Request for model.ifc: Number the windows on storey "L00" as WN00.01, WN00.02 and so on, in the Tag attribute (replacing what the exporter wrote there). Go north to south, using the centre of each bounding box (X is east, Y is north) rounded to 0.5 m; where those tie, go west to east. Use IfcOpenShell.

First a look at what the model holds.

```python
import ifcopenshell
import ifcopenshell.util.element
import ifcopenshell.util.placement

model = ifcopenshell.open("model.ifc")
print(model.schema)
storey = next(s for s in model.by_type("IfcBuildingStorey") if s.Name == "L00")
windows = [e for e in ifcopenshell.util.element.get_decomposition(storey) if e.is_a("IfcWindow")]
for e in sorted(windows, key=lambda e: e.id()):
    origin = ifcopenshell.util.placement.get_local_placement(e.ObjectPlacement)[:3, 3]
    print(e.id(), e.Tag, e.Name, origin.round(2) + 0.0, sep=" | ")
```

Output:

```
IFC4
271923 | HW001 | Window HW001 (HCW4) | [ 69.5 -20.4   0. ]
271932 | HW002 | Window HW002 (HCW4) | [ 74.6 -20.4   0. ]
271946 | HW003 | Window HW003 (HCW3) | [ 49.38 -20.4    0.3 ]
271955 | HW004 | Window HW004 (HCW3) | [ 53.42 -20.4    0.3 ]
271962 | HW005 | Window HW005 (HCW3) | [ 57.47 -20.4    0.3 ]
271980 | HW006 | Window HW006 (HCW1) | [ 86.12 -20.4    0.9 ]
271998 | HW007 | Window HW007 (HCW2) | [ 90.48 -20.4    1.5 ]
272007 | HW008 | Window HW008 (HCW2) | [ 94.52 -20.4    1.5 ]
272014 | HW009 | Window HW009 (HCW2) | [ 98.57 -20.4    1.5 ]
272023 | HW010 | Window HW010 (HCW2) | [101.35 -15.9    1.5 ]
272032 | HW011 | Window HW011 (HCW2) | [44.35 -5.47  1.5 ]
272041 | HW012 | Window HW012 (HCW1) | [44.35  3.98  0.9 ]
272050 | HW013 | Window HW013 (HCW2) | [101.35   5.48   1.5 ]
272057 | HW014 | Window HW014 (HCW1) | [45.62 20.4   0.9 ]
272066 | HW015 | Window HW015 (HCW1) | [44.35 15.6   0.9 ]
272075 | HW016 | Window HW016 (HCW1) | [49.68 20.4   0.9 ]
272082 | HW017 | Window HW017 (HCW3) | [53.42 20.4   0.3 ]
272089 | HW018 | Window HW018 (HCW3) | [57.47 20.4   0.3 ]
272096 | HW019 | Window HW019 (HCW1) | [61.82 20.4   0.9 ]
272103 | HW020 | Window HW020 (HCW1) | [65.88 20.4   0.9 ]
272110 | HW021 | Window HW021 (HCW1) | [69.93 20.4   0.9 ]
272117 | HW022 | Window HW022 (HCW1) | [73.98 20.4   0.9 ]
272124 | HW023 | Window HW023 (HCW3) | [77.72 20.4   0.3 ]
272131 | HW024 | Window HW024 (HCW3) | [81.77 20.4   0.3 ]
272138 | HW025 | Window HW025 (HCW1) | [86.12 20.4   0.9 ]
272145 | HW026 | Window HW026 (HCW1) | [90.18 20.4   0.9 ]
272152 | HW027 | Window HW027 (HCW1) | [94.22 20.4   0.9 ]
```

```python
import ifcopenshell
import ifcopenshell.geom
import ifcopenshell.util.element
import ifcopenshell.util.shape

model = ifcopenshell.open("model.ifc")
settings = ifcopenshell.geom.settings()
settings.set("use-world-coords", True)


def centre(element):
    shape = ifcopenshell.geom.create_shape(settings, element)
    return ifcopenshell.util.shape.get_bbox_centroid(shape.geometry)


storey = next(s for s in model.by_type("IfcBuildingStorey") if s.Name == "L00")
windows = [e for e in ifcopenshell.util.element.get_decomposition(storey) if e.is_a("IfcWindow")]

# Insertion points can sit at a corner or the storey origin, so sort by the geometry (in metres).
centres = {e: centre(e) for e in windows}
windows.sort(key=lambda e: (-round(centres[e][1] / 0.5), centres[e][0]))

for i, e in enumerate(windows, start=1):
    number = f"WN00.{i:02d}"
    e.Tag = number
    print(e.id(), number)

model.write("model_v2.ifc")
```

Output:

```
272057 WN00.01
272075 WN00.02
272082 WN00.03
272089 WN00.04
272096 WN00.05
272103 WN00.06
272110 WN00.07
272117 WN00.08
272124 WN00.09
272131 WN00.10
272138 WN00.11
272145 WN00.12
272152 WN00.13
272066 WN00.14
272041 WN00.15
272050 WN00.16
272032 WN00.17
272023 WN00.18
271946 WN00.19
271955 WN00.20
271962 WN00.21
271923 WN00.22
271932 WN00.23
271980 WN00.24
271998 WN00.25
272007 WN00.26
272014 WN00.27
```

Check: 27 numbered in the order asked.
